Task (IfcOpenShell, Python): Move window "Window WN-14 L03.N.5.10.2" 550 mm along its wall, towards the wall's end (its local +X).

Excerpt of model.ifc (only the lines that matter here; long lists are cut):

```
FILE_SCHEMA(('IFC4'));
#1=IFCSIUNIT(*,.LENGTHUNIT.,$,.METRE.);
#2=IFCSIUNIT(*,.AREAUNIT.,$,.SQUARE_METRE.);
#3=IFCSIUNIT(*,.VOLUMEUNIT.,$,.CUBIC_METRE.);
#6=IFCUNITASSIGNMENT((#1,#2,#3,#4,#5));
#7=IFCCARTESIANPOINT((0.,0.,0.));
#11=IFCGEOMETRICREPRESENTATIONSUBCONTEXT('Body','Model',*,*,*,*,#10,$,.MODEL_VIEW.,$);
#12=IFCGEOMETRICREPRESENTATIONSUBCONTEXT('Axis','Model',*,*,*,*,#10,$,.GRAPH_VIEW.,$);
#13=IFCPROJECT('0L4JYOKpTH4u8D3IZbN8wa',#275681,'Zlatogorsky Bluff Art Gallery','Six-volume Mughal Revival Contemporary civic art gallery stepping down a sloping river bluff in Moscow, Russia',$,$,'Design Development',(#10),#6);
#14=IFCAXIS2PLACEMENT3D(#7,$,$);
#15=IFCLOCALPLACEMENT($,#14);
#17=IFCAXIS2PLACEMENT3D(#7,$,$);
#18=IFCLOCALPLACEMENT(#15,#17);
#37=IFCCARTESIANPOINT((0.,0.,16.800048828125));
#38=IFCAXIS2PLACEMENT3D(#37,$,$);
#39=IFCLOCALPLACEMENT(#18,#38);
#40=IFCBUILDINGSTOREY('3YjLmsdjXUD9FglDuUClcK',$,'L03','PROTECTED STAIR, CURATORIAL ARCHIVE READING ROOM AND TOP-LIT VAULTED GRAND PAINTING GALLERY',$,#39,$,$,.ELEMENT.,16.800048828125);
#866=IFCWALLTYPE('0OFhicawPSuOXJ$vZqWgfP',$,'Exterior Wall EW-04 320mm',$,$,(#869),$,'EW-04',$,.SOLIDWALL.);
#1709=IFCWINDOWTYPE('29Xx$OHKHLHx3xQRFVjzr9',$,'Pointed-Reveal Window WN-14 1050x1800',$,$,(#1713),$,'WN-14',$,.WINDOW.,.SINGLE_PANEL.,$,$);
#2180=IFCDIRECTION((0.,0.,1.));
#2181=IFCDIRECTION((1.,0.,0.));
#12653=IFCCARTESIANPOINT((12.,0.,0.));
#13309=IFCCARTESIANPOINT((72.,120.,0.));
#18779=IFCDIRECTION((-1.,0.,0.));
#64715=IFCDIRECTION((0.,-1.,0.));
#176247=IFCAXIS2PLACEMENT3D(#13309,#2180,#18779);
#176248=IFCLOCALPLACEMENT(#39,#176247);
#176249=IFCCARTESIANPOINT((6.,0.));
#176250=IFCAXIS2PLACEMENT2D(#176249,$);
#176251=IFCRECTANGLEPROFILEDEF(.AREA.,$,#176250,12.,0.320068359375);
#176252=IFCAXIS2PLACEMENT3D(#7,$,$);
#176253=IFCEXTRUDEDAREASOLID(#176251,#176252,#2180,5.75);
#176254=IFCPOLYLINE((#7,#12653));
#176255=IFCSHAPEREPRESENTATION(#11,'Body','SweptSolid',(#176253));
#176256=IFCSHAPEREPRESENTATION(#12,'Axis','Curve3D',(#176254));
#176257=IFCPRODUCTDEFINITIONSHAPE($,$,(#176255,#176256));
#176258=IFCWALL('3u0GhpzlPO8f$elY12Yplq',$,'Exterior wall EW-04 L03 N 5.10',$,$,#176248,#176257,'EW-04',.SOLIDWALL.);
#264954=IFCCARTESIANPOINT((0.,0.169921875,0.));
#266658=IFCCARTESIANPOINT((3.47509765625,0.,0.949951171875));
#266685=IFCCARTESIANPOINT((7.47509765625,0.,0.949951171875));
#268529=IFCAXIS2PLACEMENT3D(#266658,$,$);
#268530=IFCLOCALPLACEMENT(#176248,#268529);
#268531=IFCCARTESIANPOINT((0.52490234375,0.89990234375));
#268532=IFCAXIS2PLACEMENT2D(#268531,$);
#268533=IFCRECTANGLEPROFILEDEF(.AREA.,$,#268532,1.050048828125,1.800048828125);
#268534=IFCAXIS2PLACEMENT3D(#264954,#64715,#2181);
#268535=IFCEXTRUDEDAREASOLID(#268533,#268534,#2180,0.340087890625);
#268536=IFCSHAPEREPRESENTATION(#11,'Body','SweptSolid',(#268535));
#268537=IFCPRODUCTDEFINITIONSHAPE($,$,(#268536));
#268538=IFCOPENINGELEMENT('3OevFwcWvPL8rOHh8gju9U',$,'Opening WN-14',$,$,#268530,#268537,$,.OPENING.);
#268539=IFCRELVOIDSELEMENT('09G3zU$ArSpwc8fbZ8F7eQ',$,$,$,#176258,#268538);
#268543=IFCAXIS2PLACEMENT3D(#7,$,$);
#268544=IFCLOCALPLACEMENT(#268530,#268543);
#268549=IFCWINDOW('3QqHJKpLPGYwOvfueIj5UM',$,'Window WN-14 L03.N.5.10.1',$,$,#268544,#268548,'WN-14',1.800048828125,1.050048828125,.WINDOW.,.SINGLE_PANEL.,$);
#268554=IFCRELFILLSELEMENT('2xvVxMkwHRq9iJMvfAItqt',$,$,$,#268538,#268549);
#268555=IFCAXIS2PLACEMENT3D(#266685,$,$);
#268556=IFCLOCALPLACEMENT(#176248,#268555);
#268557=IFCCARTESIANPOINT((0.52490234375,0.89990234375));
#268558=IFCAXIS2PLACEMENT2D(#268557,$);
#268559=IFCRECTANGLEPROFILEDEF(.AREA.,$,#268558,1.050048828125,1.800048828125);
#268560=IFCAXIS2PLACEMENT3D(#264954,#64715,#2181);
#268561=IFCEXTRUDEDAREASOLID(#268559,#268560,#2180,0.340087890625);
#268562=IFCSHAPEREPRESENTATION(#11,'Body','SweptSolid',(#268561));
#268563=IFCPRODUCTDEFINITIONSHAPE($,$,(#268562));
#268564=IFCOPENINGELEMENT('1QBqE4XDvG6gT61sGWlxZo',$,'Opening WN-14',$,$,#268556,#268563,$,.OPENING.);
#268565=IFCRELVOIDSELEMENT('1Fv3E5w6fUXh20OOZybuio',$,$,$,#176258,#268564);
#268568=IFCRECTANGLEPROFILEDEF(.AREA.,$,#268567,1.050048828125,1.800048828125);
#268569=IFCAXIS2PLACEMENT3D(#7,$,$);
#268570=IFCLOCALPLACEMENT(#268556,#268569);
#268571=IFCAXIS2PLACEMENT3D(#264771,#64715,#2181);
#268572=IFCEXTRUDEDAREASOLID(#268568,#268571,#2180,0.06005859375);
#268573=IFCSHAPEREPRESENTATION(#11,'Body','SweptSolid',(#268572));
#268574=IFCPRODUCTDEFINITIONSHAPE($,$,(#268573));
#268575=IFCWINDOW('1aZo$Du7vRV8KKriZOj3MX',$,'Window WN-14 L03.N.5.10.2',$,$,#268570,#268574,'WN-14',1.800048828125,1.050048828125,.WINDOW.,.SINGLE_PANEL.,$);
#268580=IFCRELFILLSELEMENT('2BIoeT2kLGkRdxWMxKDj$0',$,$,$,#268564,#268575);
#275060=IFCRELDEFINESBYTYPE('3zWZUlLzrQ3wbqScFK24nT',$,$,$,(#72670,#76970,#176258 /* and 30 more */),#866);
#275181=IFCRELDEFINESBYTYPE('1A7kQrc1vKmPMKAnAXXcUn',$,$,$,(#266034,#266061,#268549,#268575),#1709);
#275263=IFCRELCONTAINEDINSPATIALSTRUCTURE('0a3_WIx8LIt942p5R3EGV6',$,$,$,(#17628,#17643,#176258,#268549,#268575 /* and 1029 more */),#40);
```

```python
import ifcopenshell
import ifcopenshell.api.geometry
import ifcopenshell.util.placement
import ifcopenshell.util.unit

model = ifcopenshell.open("model.ifc")
unit_scale = ifcopenshell.util.unit.calculate_unit_scale(model)

window = model.by_guid("1aZo$Du7vRV8KKriZOj3MX")
opening = window.FillsVoids[0].RelatingOpeningElement
wall = opening.VoidsElements[0].RelatingBuildingElement

wall_matrix = ifcopenshell.util.placement.get_local_placement(wall.ObjectPlacement)
shift = wall_matrix[:3, 0] * 0.55 / unit_scale
before = ifcopenshell.util.placement.get_local_placement(window.ObjectPlacement)[:3, 3].copy()

# The window is placed relative to its opening, so it follows when the opening moves.
matrix = ifcopenshell.util.placement.get_local_placement(opening.ObjectPlacement)
matrix[:3, 3] += shift
ifcopenshell.api.geometry.edit_object_placement(
    model, product=opening, matrix=matrix, is_si=False, should_transform_children=True
)

after = ifcopenshell.util.placement.get_local_placement(window.ObjectPlacement)[:3, 3]
print("window moved by", (after - before).round(3) + 0.0)

model.write("model_rev.ifc")
```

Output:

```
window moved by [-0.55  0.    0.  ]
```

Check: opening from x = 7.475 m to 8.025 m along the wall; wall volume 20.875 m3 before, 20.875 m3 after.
